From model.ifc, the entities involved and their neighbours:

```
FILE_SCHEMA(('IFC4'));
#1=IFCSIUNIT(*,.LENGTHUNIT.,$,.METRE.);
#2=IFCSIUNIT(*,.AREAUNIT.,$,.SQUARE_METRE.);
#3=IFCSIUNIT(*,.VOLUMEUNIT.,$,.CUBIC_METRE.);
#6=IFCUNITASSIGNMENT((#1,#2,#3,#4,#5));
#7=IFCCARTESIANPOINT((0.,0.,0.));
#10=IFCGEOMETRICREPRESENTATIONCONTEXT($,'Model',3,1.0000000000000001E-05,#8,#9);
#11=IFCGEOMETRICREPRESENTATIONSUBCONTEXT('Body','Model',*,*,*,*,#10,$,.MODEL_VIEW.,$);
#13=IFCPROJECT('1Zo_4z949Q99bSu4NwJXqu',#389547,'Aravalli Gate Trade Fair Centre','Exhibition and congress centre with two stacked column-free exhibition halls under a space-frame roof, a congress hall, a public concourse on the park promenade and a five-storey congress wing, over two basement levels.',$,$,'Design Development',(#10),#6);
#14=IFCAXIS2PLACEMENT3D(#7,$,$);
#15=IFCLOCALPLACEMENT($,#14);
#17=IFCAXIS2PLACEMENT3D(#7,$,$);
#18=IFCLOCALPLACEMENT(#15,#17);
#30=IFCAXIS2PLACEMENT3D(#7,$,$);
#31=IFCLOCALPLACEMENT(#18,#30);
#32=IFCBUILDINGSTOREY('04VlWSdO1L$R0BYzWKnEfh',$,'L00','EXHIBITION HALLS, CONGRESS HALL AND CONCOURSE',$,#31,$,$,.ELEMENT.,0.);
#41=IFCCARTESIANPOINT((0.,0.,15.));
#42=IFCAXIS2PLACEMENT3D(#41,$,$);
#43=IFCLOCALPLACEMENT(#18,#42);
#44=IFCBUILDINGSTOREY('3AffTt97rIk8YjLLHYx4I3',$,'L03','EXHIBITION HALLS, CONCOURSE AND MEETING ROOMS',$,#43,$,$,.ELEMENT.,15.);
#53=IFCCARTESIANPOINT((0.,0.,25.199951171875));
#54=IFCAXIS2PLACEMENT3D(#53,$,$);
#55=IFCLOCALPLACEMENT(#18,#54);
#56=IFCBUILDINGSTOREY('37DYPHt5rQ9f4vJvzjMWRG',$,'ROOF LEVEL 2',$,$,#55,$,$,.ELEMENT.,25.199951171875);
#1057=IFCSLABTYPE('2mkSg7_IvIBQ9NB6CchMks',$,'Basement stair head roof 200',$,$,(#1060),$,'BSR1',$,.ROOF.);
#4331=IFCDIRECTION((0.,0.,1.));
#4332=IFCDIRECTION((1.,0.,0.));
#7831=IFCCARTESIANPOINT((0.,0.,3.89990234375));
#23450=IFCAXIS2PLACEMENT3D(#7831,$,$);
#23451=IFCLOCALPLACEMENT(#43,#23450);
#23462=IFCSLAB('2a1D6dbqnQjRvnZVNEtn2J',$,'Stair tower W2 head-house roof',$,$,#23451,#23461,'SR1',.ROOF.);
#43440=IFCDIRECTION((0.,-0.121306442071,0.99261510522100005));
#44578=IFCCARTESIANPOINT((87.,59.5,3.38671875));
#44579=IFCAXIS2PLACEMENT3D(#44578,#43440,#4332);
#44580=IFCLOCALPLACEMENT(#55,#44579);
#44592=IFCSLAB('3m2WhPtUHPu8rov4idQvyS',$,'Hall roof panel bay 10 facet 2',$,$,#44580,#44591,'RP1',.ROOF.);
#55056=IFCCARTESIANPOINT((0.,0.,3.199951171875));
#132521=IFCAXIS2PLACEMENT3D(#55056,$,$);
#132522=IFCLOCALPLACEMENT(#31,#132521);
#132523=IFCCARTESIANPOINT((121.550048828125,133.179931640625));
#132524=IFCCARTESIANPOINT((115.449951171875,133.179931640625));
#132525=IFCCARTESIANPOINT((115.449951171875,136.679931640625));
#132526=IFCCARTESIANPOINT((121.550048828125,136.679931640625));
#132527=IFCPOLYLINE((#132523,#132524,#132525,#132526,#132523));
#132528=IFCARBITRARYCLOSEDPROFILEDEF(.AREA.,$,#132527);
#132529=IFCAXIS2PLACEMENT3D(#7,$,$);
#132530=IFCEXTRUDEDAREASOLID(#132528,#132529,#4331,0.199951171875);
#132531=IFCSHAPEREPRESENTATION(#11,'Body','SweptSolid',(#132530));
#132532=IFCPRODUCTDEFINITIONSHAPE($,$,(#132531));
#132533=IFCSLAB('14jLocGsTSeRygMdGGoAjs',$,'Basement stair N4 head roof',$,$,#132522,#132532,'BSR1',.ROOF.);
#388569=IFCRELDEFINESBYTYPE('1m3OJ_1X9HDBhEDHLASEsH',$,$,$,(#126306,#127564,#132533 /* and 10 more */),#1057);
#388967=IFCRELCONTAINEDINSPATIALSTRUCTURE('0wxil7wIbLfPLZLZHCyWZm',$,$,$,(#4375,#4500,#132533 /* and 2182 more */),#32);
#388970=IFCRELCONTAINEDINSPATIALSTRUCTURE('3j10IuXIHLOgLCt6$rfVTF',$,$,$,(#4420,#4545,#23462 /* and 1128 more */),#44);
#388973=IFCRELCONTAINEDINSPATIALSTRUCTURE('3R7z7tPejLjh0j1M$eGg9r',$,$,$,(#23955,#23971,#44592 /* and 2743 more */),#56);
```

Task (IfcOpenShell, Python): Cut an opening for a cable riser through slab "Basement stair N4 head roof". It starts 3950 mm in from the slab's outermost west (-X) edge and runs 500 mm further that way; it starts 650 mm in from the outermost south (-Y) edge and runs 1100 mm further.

```python
import numpy as np
import ifcopenshell
import ifcopenshell.api.feature
import ifcopenshell.api.geometry
import ifcopenshell.api.root
import ifcopenshell.geom
import ifcopenshell.util.placement
import ifcopenshell.util.representation
import ifcopenshell.util.shape
import ifcopenshell.util.unit

model = ifcopenshell.open("model.ifc")
unit_scale = ifcopenshell.util.unit.calculate_unit_scale(model)
settings = ifcopenshell.geom.settings()


def volume(element):
    """Net volume in cubic metres, openings subtracted."""
    shape = ifcopenshell.geom.create_shape(settings, element)
    return ifcopenshell.util.shape.get_volume(shape.geometry)


slab = model.by_guid("14jLocGsTSeRygMdGGoAjs")
before = volume(slab)

# Extent in the slab's own axes, in metres. The edges named are its -X and -Y sides.
slab_shape = ifcopenshell.geom.create_shape(settings, slab)
vertices = ifcopenshell.util.shape.get_vertices(slab_shape.geometry)
x_min, y_min, bottom = vertices.min(axis=0)
top = vertices[:, 2].max()

opening = ifcopenshell.api.root.create_entity(model, ifc_class="IfcOpeningElement", name="Cable riser opening", predefined_type="OPENING")
context = ifcopenshell.util.representation.get_context(model, "Model", "Body", "MODEL_VIEW")
width, depth = 0.5, 1.1
outline = [(0.0, 0.0), (width, 0.0), (width, depth), (0.0, depth), (0.0, 0.0)]
# Overshoot both faces by 50 mm so the cut is clean.
shape = ifcopenshell.api.geometry.add_slab_representation(
    model, context=context, depth=top - bottom + 0.1, polyline=outline
)
ifcopenshell.api.geometry.assign_representation(model, product=opening, representation=shape)

matrix = ifcopenshell.util.placement.get_local_placement(slab.ObjectPlacement)
matrix[:, 3] = matrix @ np.append(np.array([x_min + 3.95, y_min + 0.65, bottom - 0.05]) / unit_scale, 1.0)
ifcopenshell.api.geometry.edit_object_placement(model, product=opening, matrix=matrix, is_si=False)
ifcopenshell.api.feature.add_feature(model, feature=opening, element=slab)

after = volume(slab)

print(f"slab volume {before:.3f} -> {after:.3f} m3")

model.write("model_v2.ifc")
```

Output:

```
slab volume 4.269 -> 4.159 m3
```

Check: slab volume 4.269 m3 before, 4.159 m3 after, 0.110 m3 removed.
